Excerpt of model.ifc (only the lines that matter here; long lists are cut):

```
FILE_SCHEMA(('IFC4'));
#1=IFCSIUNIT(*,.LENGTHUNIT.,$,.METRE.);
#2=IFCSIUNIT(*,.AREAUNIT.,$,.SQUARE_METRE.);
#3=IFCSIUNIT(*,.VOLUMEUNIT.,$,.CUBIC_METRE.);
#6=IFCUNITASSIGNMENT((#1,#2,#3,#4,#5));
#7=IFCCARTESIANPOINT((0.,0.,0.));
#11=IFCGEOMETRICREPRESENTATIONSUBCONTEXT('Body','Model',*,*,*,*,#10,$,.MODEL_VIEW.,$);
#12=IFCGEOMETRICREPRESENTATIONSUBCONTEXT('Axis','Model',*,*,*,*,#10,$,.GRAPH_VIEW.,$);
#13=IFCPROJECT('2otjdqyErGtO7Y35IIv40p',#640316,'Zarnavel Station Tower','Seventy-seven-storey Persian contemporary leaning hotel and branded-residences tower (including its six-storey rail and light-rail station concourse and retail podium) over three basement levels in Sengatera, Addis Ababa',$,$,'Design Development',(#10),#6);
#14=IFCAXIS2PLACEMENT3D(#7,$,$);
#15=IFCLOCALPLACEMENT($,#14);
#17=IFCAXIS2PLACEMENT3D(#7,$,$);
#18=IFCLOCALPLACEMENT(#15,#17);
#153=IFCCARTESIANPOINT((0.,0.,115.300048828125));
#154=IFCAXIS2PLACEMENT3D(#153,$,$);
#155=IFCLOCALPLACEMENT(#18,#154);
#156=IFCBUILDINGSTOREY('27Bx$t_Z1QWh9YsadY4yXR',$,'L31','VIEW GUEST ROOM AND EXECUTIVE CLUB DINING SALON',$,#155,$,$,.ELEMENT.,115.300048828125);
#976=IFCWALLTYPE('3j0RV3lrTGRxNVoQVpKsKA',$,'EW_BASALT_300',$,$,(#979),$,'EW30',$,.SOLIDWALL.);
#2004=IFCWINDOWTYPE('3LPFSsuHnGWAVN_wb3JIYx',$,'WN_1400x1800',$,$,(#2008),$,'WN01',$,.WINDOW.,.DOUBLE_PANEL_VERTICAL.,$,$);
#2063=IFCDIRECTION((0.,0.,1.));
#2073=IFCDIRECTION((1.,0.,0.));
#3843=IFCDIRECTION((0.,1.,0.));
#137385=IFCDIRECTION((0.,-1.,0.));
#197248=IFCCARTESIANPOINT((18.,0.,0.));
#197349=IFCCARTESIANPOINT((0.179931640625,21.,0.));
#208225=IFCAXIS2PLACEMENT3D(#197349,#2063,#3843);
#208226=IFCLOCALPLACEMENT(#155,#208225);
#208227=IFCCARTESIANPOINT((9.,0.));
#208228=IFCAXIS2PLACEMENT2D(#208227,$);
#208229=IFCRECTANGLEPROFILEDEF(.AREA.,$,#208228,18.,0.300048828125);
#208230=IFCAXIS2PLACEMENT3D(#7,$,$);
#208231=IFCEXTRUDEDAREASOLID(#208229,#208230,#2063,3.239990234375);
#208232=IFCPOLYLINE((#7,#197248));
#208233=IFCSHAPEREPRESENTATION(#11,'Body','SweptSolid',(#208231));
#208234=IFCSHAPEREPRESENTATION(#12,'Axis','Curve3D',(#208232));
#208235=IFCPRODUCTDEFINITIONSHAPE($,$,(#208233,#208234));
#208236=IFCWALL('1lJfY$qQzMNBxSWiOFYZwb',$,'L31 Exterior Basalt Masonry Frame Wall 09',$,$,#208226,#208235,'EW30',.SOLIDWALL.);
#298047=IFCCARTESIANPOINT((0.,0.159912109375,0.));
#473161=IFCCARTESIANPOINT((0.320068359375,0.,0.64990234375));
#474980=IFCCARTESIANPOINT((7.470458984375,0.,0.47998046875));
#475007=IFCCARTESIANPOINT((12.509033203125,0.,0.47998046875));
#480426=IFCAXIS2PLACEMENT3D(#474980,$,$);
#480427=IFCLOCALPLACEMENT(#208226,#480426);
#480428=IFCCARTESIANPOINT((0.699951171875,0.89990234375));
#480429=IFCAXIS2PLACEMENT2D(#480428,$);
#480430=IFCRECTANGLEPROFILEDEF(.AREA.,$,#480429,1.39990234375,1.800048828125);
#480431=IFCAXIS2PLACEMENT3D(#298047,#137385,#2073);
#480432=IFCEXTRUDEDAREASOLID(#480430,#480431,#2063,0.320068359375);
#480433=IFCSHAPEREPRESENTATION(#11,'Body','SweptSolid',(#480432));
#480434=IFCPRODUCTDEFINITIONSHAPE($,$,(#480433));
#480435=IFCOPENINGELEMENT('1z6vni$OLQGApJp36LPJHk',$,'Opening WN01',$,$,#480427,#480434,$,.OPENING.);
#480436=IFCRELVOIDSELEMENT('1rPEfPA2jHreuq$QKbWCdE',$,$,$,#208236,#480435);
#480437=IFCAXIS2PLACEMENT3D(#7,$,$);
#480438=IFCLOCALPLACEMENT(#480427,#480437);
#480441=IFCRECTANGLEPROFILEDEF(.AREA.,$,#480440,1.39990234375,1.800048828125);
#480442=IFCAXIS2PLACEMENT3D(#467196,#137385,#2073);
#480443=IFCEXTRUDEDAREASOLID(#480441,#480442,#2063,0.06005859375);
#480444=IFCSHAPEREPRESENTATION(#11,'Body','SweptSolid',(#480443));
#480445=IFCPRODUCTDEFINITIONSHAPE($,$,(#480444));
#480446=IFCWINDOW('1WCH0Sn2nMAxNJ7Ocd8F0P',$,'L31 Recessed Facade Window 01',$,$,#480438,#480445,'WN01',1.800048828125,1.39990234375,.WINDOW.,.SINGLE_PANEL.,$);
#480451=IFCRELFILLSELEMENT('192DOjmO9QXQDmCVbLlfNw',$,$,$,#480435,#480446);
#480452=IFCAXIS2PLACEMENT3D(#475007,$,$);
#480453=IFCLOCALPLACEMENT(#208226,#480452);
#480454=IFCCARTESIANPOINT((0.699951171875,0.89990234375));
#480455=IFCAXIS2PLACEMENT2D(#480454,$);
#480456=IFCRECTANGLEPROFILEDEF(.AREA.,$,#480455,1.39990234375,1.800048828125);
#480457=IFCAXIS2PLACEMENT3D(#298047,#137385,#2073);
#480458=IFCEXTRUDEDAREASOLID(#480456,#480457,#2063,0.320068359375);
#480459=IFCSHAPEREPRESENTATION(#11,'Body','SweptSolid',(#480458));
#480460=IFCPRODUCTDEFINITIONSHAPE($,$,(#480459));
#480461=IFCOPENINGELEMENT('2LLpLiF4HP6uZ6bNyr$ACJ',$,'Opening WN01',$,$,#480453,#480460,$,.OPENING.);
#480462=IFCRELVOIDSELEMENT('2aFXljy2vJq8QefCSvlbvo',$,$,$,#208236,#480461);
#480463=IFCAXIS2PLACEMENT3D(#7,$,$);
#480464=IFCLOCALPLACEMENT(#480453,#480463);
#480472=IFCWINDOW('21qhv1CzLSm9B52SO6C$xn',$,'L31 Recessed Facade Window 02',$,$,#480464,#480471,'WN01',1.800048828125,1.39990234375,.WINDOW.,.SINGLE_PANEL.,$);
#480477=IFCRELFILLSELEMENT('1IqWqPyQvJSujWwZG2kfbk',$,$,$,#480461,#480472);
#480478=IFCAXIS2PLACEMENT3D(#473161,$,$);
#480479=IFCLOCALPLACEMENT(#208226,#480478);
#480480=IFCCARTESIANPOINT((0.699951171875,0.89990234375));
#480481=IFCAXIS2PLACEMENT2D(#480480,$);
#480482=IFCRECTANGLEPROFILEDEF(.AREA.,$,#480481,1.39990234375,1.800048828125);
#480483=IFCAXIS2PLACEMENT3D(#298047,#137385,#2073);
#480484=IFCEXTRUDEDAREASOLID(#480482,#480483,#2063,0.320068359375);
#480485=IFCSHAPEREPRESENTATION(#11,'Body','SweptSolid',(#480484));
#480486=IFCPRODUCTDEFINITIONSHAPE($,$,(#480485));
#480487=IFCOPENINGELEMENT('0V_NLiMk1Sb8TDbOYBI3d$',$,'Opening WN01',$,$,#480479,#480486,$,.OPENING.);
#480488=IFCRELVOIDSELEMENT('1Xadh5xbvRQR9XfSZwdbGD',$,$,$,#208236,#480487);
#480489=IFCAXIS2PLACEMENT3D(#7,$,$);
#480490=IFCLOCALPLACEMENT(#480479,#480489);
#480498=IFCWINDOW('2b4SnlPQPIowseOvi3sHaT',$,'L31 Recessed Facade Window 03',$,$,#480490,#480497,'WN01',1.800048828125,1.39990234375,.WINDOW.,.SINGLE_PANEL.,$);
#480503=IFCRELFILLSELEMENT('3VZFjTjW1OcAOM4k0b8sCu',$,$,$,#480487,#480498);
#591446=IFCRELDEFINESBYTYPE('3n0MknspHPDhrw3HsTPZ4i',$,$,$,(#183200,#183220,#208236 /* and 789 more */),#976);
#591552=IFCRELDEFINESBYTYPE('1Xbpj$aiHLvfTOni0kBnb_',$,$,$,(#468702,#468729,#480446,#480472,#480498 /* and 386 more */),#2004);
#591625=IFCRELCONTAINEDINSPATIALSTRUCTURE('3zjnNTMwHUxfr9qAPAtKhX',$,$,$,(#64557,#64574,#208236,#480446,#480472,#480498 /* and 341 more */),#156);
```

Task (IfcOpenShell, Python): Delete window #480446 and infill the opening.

```python
import ifcopenshell
import ifcopenshell.api.feature
import ifcopenshell.api.root
import ifcopenshell.geom
import ifcopenshell.util.shape

model = ifcopenshell.open("model.ifc")
settings = ifcopenshell.geom.settings()


def volume(element):
    """Net volume in cubic metres, openings subtracted."""
    shape = ifcopenshell.geom.create_shape(settings, element)
    return ifcopenshell.util.shape.get_volume(shape.geometry)


window = model.by_guid("1WCH0Sn2nMAxNJ7Ocd8F0P")
opening = window.FillsVoids[0].RelatingOpeningElement
wall = opening.VoidsElements[0].RelatingBuildingElement
before = volume(wall)

ifcopenshell.api.root.remove_product(model, product=window)
ifcopenshell.api.feature.remove_feature(model, feature=opening)

after = volume(wall)

print(f"wall volume {before:.3f} -> {after:.3f} m3")

model.write("model_v2.ifc")
```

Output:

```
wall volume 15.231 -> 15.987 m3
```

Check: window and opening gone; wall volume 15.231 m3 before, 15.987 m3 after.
